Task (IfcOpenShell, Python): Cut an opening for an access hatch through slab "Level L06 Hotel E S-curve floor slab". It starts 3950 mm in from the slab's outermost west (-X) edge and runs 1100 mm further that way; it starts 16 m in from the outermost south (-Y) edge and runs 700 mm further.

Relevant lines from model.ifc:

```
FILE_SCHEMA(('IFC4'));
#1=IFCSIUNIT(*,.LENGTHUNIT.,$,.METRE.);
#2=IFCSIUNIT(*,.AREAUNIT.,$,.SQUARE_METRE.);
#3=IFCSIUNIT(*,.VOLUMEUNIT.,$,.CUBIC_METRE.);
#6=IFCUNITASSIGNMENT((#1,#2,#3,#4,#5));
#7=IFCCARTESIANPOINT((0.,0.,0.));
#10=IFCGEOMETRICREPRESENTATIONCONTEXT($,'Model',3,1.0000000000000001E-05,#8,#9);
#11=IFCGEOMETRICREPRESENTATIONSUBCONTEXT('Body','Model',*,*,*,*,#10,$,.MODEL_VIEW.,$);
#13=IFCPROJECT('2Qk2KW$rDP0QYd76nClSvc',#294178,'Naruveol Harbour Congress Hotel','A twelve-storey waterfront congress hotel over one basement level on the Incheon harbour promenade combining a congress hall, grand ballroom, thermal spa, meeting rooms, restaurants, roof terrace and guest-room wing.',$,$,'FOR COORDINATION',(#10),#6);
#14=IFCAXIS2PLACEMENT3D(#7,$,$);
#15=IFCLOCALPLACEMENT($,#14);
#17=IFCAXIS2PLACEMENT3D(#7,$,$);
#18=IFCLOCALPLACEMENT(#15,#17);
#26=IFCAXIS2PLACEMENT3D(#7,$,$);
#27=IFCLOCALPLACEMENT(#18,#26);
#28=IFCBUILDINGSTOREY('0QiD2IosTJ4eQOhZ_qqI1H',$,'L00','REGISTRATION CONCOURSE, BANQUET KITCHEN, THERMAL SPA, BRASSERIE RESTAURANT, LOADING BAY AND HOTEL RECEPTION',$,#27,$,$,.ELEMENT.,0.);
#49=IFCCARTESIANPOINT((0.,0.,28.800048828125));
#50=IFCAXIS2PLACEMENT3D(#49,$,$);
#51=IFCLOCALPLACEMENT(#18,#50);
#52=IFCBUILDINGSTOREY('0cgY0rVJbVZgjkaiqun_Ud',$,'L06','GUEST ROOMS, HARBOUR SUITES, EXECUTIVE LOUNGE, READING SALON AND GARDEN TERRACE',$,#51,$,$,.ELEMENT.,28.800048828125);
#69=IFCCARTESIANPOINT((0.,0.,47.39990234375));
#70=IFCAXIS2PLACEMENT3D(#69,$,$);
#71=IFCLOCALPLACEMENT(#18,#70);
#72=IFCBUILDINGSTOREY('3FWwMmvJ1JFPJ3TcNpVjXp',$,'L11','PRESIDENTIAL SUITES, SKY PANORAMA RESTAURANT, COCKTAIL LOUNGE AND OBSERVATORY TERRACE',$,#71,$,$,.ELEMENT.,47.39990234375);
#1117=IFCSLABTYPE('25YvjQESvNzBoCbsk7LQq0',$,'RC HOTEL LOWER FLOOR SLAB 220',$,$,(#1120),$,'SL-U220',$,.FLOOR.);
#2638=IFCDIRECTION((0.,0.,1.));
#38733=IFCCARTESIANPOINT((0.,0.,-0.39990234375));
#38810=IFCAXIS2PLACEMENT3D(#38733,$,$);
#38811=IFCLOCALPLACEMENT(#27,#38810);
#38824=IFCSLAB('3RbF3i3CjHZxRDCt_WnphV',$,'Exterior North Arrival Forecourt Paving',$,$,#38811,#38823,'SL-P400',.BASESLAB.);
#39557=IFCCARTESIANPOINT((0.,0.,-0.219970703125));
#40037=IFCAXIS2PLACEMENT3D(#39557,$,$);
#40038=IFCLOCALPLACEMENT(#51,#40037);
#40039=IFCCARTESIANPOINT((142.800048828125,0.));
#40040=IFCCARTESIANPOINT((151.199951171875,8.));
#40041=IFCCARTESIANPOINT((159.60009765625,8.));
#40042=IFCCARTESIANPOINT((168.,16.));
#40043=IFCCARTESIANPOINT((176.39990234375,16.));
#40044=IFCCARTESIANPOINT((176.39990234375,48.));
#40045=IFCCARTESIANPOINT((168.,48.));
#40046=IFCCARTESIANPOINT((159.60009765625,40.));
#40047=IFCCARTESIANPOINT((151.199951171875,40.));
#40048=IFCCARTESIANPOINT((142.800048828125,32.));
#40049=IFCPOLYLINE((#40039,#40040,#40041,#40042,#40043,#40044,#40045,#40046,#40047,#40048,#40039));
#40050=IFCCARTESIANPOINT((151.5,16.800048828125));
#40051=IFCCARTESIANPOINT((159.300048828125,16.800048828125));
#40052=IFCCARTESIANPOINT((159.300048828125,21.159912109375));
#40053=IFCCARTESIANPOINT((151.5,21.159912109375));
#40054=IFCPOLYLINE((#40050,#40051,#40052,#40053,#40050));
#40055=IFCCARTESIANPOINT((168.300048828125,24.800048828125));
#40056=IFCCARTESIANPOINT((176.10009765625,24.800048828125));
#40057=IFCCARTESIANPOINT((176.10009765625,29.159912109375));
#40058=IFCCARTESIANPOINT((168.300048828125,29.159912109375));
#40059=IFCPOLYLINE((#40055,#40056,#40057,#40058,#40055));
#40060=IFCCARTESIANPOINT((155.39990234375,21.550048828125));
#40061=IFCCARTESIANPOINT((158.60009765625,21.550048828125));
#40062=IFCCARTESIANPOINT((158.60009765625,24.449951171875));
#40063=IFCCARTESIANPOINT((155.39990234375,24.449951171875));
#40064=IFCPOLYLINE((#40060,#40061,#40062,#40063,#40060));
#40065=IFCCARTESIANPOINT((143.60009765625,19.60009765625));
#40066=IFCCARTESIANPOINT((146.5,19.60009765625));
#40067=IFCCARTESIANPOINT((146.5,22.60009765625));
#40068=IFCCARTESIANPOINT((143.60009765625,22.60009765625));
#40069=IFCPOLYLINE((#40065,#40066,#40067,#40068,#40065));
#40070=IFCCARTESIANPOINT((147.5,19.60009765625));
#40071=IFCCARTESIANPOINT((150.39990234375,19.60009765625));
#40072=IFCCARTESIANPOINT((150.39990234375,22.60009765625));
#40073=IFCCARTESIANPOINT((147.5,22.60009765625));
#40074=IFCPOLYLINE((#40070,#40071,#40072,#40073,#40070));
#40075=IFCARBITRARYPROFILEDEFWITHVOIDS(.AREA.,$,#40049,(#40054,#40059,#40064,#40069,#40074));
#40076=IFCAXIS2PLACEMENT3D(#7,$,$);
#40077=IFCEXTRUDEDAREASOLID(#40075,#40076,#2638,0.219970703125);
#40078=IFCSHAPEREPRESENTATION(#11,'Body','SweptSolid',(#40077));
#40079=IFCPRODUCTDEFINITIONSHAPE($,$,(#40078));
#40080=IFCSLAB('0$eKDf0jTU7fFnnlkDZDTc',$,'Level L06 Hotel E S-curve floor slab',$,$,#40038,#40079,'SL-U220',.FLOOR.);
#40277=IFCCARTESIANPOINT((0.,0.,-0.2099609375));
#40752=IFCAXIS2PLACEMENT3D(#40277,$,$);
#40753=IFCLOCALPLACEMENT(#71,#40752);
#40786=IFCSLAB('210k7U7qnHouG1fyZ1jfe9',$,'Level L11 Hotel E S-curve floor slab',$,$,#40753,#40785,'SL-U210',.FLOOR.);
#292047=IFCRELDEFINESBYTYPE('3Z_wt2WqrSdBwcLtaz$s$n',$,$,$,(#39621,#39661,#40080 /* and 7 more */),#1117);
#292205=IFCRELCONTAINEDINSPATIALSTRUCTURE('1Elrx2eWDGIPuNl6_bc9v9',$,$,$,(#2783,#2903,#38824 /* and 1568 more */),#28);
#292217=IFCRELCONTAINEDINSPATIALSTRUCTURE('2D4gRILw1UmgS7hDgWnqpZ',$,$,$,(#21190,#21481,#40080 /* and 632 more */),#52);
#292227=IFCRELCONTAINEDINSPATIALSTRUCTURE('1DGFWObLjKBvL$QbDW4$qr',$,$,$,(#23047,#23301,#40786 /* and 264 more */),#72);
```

```python
import numpy as np
import ifcopenshell
import ifcopenshell.api.feature
import ifcopenshell.api.geometry
import ifcopenshell.api.root
import ifcopenshell.geom
import ifcopenshell.util.placement
import ifcopenshell.util.representation
import ifcopenshell.util.shape
import ifcopenshell.util.unit

model = ifcopenshell.open("model.ifc")
unit_scale = ifcopenshell.util.unit.calculate_unit_scale(model)
settings = ifcopenshell.geom.settings()


def volume(element):
    """Net volume in cubic metres, openings subtracted."""
    shape = ifcopenshell.geom.create_shape(settings, element)
    return ifcopenshell.util.shape.get_volume(shape.geometry)


slab = model.by_guid("0$eKDf0jTU7fFnnlkDZDTc")
before = volume(slab)

# Extent in the slab's own axes, in metres. The edges named are its -X and -Y sides.
slab_shape = ifcopenshell.geom.create_shape(settings, slab)
vertices = ifcopenshell.util.shape.get_vertices(slab_shape.geometry)
x_min, y_min, bottom = vertices.min(axis=0)
top = vertices[:, 2].max()

opening = ifcopenshell.api.root.create_entity(model, ifc_class="IfcOpeningElement", name="Access hatch opening", predefined_type="OPENING")
context = ifcopenshell.util.representation.get_context(model, "Model", "Body", "MODEL_VIEW")
width, depth = 1.1, 0.7
outline = [(0.0, 0.0), (width, 0.0), (width, depth), (0.0, depth), (0.0, 0.0)]
# Overshoot both faces by 50 mm so the cut is clean.
shape = ifcopenshell.api.geometry.add_slab_representation(
    model, context=context, depth=top - bottom + 0.1, polyline=outline
)
ifcopenshell.api.geometry.assign_representation(model, product=opening, representation=shape)

matrix = ifcopenshell.util.placement.get_local_placement(slab.ObjectPlacement)
matrix[:, 3] = matrix @ np.append(np.array([x_min + 3.95, y_min + 16, bottom - 0.05]) / unit_scale, 1.0)
ifcopenshell.api.geometry.edit_object_placement(model, product=opening, matrix=matrix, is_si=False)
ifcopenshell.api.feature.add_feature(model, feature=opening, element=slab)

after = volume(slab)

print(f"slab volume {before:.3f} -> {after:.3f} m3")

model.write("model_v2.ifc")
```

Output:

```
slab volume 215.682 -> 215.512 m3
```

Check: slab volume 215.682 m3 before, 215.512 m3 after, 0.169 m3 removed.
